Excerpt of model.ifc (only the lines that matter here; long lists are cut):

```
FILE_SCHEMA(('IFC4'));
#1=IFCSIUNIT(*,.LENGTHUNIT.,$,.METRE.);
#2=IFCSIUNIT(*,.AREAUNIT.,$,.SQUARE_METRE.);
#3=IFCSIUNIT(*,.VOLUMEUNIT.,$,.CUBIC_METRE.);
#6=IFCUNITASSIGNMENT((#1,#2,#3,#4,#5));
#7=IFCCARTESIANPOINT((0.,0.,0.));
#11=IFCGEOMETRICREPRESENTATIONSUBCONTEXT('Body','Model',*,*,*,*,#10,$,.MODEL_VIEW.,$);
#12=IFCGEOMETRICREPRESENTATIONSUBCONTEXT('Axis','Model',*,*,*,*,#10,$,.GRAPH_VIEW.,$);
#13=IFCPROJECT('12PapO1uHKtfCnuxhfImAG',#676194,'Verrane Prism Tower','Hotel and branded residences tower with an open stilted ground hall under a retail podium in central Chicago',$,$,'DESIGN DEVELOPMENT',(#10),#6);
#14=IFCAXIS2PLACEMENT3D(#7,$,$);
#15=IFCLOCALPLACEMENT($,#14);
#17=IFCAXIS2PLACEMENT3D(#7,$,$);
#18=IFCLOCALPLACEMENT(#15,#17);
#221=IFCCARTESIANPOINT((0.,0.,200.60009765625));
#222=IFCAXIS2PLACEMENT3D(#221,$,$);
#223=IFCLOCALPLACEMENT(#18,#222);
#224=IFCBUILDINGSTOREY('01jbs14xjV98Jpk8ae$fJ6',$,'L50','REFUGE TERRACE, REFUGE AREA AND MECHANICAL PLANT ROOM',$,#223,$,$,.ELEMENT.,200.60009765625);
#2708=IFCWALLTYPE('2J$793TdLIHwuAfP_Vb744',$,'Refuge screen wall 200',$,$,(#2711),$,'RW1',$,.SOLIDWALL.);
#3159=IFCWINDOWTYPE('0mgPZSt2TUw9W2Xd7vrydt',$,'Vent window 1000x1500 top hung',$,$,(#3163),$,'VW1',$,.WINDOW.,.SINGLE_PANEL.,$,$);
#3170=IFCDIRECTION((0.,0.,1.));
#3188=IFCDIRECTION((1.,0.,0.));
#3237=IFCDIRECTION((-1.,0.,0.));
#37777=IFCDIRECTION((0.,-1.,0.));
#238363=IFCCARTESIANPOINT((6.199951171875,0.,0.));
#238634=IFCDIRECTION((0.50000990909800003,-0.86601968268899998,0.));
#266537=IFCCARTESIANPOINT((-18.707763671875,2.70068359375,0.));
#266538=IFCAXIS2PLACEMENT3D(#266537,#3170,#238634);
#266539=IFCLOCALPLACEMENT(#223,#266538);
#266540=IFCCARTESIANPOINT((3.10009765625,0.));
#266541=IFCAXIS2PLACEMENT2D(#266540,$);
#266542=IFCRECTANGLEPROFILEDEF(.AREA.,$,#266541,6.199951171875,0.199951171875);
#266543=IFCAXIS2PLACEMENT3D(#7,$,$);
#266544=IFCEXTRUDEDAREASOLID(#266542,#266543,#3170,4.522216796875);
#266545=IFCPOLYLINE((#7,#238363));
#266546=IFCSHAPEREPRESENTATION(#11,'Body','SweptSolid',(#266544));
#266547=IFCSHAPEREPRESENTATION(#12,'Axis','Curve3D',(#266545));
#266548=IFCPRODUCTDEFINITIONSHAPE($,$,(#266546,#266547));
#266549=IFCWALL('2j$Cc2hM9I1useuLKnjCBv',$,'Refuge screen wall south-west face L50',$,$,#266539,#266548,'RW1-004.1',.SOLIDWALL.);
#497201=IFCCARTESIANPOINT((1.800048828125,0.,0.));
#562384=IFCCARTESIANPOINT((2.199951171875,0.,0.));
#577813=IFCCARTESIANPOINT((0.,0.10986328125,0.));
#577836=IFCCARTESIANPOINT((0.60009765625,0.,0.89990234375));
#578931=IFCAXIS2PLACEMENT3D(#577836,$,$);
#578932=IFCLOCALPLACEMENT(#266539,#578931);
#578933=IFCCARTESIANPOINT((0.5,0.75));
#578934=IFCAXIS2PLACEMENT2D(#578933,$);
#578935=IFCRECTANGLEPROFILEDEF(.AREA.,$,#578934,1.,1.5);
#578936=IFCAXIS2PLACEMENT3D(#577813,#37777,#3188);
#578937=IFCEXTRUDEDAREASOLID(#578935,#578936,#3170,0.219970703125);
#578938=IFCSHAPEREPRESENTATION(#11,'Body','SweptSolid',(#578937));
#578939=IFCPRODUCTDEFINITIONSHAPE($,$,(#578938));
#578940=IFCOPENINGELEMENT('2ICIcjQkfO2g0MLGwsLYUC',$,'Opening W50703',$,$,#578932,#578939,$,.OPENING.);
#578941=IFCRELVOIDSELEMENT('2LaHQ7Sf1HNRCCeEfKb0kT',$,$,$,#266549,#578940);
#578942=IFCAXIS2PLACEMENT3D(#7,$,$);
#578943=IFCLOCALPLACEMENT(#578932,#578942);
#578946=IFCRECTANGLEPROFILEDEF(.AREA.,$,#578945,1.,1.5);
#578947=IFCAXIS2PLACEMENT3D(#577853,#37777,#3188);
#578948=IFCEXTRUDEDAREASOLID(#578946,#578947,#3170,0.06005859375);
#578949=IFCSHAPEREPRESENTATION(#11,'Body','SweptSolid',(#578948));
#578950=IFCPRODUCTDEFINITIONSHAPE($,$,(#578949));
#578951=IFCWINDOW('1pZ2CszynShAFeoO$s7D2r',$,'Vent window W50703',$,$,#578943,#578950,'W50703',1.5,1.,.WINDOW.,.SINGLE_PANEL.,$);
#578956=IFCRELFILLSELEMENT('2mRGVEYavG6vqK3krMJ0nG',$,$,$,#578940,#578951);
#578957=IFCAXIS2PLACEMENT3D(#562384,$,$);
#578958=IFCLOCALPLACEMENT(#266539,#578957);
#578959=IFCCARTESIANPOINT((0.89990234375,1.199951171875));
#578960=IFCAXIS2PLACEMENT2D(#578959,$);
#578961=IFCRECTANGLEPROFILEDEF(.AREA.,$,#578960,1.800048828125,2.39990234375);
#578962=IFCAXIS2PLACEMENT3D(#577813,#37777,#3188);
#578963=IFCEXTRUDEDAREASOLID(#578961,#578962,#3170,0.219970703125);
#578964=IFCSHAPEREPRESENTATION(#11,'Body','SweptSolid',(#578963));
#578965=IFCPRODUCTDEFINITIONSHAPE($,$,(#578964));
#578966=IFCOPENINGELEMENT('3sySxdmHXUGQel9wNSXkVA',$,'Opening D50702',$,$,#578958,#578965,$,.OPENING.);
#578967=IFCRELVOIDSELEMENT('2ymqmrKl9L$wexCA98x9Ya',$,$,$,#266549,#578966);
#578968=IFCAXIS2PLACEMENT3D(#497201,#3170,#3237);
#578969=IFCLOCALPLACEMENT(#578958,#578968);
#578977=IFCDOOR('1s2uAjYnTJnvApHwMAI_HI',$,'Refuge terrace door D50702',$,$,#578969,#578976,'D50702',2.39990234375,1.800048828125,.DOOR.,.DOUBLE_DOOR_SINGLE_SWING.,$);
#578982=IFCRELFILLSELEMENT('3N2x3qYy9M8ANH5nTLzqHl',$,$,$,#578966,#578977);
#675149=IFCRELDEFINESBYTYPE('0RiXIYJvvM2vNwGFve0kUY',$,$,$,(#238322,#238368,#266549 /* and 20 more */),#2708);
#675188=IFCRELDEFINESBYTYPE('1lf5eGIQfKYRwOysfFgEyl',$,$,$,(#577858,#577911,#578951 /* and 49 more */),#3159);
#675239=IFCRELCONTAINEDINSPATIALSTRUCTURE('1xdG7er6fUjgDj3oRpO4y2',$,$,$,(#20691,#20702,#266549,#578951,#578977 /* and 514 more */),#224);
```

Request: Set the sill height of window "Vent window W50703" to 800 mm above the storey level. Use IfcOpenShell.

```python
import numpy as np
import ifcopenshell
import ifcopenshell.api.geometry
import ifcopenshell.geom
import ifcopenshell.util.element
import ifcopenshell.util.placement
import ifcopenshell.util.shape
import ifcopenshell.util.unit

model = ifcopenshell.open("model.ifc")
unit_scale = ifcopenshell.util.unit.calculate_unit_scale(model)

window = model.by_guid("1pZ2CszynShAFeoO$s7D2r")
opening = window.FillsVoids[0].RelatingOpeningElement
storey = ifcopenshell.util.element.get_container(window, ifc_class="IfcBuildingStorey")
level = ifcopenshell.util.placement.get_local_placement(storey.ObjectPlacement)[2, 3]

# The opening's origin need not be at the sill, so measure its lowest point.
shape = ifcopenshell.geom.create_shape(ifcopenshell.geom.settings(), opening)
bottom = ifcopenshell.util.shape.get_shape_bottom_elevation(shape, shape.geometry) / unit_scale
dz = level + 0.8 - bottom

shift = np.array([0.0, 0.0, dz])
# The window is placed relative to its opening, so it follows when the opening moves.
matrix = ifcopenshell.util.placement.get_local_placement(opening.ObjectPlacement)
matrix[:3, 3] += shift
ifcopenshell.api.geometry.edit_object_placement(
    model, product=opening, matrix=matrix, is_si=False, should_transform_children=True
)

print(f"moved by {dz * unit_scale:+.3f} m")

model.write("model-out.ifc")
```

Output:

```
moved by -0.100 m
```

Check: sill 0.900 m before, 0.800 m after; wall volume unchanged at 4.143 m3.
